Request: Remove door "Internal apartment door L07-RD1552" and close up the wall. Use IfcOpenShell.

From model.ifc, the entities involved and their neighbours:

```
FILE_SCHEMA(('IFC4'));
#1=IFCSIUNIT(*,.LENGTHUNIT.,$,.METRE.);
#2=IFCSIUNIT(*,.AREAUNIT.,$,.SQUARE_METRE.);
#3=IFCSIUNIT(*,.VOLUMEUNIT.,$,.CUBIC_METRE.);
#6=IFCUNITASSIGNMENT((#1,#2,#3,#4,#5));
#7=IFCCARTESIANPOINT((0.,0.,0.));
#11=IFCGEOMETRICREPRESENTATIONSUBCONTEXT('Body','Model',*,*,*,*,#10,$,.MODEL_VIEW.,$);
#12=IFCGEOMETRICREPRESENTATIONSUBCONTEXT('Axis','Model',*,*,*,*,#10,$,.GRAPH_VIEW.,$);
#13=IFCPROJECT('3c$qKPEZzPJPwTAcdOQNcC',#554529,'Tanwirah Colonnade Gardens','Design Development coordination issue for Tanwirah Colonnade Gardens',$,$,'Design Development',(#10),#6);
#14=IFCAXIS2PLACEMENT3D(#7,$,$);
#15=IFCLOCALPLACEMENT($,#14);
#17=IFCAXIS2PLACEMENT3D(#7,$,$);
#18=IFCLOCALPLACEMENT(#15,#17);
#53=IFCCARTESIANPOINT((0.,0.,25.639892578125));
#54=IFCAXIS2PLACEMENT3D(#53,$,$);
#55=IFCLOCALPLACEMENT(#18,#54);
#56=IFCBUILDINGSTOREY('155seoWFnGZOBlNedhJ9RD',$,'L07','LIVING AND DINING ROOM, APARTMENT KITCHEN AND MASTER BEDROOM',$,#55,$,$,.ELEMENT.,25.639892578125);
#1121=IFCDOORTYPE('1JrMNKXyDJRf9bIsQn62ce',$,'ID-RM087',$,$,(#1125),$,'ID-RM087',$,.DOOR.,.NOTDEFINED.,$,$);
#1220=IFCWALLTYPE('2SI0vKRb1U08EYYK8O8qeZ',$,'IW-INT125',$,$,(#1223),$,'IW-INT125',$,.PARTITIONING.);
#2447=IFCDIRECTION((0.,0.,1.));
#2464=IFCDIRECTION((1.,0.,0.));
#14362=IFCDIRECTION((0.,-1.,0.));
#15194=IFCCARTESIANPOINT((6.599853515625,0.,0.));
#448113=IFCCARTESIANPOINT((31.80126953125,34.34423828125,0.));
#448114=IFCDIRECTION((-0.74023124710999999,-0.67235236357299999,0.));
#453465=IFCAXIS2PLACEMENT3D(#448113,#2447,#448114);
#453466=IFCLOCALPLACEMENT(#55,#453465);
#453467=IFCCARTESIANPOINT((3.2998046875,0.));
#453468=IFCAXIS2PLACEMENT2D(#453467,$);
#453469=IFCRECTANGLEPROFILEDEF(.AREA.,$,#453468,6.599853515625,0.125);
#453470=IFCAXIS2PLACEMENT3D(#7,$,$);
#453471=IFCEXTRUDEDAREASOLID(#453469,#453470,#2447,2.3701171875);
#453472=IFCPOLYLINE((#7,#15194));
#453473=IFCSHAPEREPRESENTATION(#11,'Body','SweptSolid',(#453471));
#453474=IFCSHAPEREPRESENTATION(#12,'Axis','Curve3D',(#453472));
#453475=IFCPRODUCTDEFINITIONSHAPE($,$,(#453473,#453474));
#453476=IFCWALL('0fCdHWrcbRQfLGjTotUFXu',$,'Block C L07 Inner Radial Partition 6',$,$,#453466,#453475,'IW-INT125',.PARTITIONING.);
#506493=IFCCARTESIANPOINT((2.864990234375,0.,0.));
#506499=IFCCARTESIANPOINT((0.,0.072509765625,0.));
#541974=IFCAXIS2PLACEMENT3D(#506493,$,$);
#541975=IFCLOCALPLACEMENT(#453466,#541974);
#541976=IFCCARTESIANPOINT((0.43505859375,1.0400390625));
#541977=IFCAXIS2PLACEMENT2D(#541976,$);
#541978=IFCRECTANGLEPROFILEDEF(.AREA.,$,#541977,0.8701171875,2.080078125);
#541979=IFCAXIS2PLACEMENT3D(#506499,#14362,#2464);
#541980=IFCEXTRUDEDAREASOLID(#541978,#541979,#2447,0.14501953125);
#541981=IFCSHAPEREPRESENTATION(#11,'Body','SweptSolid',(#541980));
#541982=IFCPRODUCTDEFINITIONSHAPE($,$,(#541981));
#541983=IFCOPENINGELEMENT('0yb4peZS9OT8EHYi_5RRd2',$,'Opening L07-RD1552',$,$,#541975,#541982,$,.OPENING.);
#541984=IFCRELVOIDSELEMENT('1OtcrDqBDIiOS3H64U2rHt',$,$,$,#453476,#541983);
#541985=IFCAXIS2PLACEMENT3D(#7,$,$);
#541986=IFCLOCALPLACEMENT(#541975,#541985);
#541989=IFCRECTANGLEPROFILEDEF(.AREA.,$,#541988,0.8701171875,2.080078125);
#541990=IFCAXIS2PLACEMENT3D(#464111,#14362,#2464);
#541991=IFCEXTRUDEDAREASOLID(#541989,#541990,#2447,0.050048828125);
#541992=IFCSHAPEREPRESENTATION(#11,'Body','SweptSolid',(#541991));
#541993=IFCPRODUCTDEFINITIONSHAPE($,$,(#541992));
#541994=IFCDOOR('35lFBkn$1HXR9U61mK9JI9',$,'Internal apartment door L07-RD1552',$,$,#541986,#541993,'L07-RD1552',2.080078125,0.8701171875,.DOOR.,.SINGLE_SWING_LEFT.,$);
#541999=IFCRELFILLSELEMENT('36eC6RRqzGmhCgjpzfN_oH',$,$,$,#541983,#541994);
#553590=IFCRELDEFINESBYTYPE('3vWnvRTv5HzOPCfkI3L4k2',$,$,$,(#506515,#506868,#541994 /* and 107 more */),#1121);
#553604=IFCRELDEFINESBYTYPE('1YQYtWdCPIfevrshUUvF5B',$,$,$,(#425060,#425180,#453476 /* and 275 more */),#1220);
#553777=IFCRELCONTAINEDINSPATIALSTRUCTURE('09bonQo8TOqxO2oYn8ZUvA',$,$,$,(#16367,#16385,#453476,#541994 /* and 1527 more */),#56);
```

```python
import ifcopenshell
import ifcopenshell.api.feature
import ifcopenshell.api.root
import ifcopenshell.geom
import ifcopenshell.util.shape

model = ifcopenshell.open("model.ifc")
settings = ifcopenshell.geom.settings()


def volume(element):
    """Net volume in cubic metres, openings subtracted."""
    shape = ifcopenshell.geom.create_shape(settings, element)
    return ifcopenshell.util.shape.get_volume(shape.geometry)


door = model.by_guid("35lFBkn$1HXR9U61mK9JI9")
opening = door.FillsVoids[0].RelatingOpeningElement
wall = opening.VoidsElements[0].RelatingBuildingElement
before = volume(wall)

ifcopenshell.api.root.remove_product(model, product=door)
ifcopenshell.api.feature.remove_feature(model, feature=opening)

after = volume(wall)

print(f"wall volume {before:.3f} -> {after:.3f} m3")

model.write("model_updated.ifc")
```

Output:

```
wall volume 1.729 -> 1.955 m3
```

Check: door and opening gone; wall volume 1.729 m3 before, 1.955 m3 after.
